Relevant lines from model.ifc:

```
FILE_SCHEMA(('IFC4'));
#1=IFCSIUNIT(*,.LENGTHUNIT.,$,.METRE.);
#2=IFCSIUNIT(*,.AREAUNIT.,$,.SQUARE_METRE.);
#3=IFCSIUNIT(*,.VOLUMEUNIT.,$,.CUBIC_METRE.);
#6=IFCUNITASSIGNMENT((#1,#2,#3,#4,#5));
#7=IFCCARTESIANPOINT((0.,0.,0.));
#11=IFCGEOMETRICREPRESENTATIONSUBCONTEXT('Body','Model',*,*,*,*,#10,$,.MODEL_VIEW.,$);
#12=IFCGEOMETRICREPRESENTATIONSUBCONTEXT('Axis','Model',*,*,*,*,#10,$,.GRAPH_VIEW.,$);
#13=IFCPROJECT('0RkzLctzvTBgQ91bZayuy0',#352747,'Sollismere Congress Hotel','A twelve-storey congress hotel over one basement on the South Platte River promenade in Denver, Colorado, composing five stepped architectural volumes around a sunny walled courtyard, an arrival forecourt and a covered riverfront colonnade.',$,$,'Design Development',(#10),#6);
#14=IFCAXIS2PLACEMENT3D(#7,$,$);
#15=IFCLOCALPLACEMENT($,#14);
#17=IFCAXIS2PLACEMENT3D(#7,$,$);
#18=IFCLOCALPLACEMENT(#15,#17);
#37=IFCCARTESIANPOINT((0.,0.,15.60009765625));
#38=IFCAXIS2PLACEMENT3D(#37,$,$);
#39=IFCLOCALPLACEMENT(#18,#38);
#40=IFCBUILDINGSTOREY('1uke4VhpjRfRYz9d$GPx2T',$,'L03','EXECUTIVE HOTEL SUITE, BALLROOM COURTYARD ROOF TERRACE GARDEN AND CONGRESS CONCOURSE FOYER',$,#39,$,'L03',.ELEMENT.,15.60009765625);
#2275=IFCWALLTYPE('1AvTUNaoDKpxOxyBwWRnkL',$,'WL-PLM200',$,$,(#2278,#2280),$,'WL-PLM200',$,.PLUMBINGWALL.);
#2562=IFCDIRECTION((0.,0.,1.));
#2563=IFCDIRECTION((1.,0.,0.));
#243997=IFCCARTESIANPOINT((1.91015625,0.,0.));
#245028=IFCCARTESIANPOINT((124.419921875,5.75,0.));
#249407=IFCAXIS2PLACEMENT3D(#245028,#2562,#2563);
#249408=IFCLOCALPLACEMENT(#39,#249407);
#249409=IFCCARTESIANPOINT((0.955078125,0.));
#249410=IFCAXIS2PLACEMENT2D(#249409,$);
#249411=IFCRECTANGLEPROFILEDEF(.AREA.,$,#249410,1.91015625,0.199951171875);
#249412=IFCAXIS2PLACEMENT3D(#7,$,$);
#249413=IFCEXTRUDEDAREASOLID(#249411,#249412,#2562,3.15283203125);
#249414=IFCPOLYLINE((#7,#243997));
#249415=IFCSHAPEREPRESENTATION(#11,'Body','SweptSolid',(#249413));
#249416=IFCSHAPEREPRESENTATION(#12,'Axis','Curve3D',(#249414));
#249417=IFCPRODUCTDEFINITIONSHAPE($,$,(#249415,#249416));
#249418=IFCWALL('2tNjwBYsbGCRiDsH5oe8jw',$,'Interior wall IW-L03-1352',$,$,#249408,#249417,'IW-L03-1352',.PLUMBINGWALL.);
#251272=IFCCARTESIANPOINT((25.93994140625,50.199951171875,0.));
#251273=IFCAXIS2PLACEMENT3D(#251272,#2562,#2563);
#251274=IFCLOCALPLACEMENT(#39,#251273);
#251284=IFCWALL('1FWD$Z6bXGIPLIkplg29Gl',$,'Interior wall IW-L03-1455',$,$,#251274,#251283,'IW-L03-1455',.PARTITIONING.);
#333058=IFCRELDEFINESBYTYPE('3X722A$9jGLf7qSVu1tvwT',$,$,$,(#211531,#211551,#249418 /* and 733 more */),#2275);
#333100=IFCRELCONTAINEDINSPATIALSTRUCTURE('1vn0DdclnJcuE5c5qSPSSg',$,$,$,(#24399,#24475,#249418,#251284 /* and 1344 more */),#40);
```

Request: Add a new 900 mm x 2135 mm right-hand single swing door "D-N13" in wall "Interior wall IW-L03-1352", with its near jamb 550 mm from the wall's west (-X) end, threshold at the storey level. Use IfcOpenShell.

```python
import numpy as np
import ifcopenshell
import ifcopenshell.api.feature
import ifcopenshell.api.geometry
import ifcopenshell.api.root
import ifcopenshell.api.spatial
import ifcopenshell.geom
import ifcopenshell.util.element
import ifcopenshell.util.placement
import ifcopenshell.util.representation
import ifcopenshell.util.shape
import ifcopenshell.util.unit

model = ifcopenshell.open("model.ifc")
unit_scale = ifcopenshell.util.unit.calculate_unit_scale(model)
settings = ifcopenshell.geom.settings()


def volume(element):
    """Net volume in cubic metres, openings subtracted."""
    shape = ifcopenshell.geom.create_shape(settings, element)
    return ifcopenshell.util.shape.get_volume(shape.geometry)


wall = model.by_guid("2tNjwBYsbGCRiDsH5oe8jw")
storey = ifcopenshell.util.element.get_container(wall, ifc_class="IfcBuildingStorey")
context = ifcopenshell.util.representation.get_context(model, "Model", "Body", "MODEL_VIEW")
before = volume(wall)

width, height, from_end, sill = 0.9, 2.135, 0.55, 0.0  # metres

# The wall runs along its own X axis, and the end named is its -X end.
wall_shape = ifcopenshell.geom.create_shape(settings, wall)
x, y, z = ifcopenshell.util.shape.get_vertices(wall_shape.geometry).T
start = x.min() + from_end
face, thickness = float(y.min()), float(y.max() - y.min())
wall_matrix = ifcopenshell.util.placement.get_local_placement(wall.ObjectPlacement)
level = ifcopenshell.util.placement.get_local_placement(storey.ObjectPlacement)[2, 3]


def in_wall(x, y):
    """Placement at x, y metres in the wall's axes, at sill height."""
    matrix = wall_matrix.copy()
    matrix[:, 3] = wall_matrix @ np.array([x / unit_scale, y / unit_scale, 0.0, 1.0])
    matrix[2, 3] = level + sill / unit_scale
    return matrix


# Opening: a box that overshoots both wall faces by 50 mm.
opening = ifcopenshell.api.root.create_entity(model, ifc_class="IfcOpeningElement", predefined_type="OPENING")
box = ifcopenshell.api.geometry.add_wall_representation(
    model, context=context, length=width, height=height, thickness=thickness + 0.1
)
ifcopenshell.api.geometry.assign_representation(model, product=opening, representation=box)
ifcopenshell.api.geometry.edit_object_placement(model, product=opening, matrix=in_wall(start, face - 0.05), is_si=False)
ifcopenshell.api.feature.add_feature(model, feature=opening, element=wall)

door = ifcopenshell.api.root.create_entity(model, ifc_class="IfcDoor", name="D-N13", predefined_type="DOOR")
door.OverallWidth, door.OverallHeight = width / unit_scale, height / unit_scale
door.OperationType = "SINGLE_SWING_RIGHT"
body = ifcopenshell.api.geometry.add_door_representation(
    model,
    context=context,
    overall_width=door.OverallWidth,
    overall_height=door.OverallHeight,
    operation_type="SINGLE_SWING_RIGHT",
    lining_properties={"LiningDepth": thickness / unit_scale, "ThresholdDepth": thickness / unit_scale},
)
ifcopenshell.api.geometry.assign_representation(model, product=door, representation=body)
ifcopenshell.api.spatial.assign_container(model, products=[door], relating_structure=storey)
ifcopenshell.api.feature.add_filling(model, opening=opening, element=door)

# The lining spans the wall, so the door starts at the wall face.
ifcopenshell.api.geometry.edit_object_placement(model, product=door, matrix=in_wall(start, face), is_si=False)

after = volume(wall)

print(f"wall volume {before:.3f} -> {after:.3f} m3")

model.write("model-out.ifc")
```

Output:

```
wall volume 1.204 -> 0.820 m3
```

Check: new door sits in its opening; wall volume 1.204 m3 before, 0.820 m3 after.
